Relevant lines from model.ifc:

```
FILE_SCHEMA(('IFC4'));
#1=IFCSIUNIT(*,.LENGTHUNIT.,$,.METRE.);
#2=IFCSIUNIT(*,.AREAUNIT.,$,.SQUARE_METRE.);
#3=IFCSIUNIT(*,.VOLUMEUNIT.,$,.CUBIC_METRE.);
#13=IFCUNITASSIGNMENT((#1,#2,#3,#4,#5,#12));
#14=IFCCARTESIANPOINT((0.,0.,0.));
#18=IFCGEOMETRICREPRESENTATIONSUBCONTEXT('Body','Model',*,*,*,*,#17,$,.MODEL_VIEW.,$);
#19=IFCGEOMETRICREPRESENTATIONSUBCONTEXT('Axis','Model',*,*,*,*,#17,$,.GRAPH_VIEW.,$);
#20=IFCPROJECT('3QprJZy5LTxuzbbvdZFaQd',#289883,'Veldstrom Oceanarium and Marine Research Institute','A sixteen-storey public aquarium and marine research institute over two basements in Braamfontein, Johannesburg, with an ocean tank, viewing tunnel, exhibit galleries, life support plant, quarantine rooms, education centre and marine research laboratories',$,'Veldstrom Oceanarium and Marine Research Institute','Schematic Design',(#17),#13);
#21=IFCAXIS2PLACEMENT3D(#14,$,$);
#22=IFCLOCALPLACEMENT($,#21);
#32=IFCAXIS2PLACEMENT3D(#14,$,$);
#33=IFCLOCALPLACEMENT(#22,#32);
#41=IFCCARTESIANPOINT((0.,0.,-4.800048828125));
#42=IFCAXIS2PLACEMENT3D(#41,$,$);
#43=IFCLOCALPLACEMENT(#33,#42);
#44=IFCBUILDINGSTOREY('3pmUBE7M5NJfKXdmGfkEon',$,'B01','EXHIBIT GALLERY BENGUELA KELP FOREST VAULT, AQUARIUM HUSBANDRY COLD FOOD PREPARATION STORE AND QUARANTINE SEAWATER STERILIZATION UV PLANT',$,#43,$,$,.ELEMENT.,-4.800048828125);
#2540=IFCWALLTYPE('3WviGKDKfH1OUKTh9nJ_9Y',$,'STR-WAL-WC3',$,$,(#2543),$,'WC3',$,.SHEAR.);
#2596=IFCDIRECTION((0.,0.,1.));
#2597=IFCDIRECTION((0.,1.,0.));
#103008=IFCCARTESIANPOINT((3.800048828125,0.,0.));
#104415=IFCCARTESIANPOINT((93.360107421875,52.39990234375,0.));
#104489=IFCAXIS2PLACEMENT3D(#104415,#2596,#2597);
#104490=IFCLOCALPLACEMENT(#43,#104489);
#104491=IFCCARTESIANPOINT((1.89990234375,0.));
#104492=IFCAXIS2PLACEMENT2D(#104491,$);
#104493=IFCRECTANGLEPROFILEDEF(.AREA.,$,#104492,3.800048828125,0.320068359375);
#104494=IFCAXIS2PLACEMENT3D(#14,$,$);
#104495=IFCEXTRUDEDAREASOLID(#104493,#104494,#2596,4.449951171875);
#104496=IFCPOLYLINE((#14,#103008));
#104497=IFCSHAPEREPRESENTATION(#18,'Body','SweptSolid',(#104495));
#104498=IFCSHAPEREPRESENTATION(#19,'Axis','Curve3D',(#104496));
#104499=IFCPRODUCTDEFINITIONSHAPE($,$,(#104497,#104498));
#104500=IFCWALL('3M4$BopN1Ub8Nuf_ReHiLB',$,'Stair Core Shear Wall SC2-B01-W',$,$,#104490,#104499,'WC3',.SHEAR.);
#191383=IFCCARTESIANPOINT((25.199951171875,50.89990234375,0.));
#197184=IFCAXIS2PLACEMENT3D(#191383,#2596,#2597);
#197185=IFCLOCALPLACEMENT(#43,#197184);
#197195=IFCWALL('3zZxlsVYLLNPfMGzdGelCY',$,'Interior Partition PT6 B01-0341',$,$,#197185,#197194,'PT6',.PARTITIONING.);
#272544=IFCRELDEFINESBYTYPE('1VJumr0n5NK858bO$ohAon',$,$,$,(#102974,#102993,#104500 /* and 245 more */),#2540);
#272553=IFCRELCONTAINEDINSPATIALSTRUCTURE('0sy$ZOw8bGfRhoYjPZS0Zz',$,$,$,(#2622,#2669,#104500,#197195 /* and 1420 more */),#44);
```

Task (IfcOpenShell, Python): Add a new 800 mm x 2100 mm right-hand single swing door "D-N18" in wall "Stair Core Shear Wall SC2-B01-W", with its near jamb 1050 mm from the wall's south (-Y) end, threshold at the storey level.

```python
import numpy as np
import ifcopenshell
import ifcopenshell.api.feature
import ifcopenshell.api.geometry
import ifcopenshell.api.root
import ifcopenshell.api.spatial
import ifcopenshell.geom
import ifcopenshell.util.element
import ifcopenshell.util.placement
import ifcopenshell.util.representation
import ifcopenshell.util.shape
import ifcopenshell.util.unit

model = ifcopenshell.open("model.ifc")
unit_scale = ifcopenshell.util.unit.calculate_unit_scale(model)
settings = ifcopenshell.geom.settings()


def volume(element):
    """Net volume in cubic metres, openings subtracted."""
    shape = ifcopenshell.geom.create_shape(settings, element)
    return ifcopenshell.util.shape.get_volume(shape.geometry)


wall = model.by_guid("3M4$BopN1Ub8Nuf_ReHiLB")
storey = ifcopenshell.util.element.get_container(wall, ifc_class="IfcBuildingStorey")
context = ifcopenshell.util.representation.get_context(model, "Model", "Body", "MODEL_VIEW")
before = volume(wall)

width, height, from_end, sill = 0.8, 2.1, 1.05, 0.0  # metres

# The wall runs along its own X axis, and the end named is its -X end.
wall_shape = ifcopenshell.geom.create_shape(settings, wall)
x, y, z = ifcopenshell.util.shape.get_vertices(wall_shape.geometry).T
start = x.min() + from_end
face, thickness = float(y.min()), float(y.max() - y.min())
wall_matrix = ifcopenshell.util.placement.get_local_placement(wall.ObjectPlacement)
level = ifcopenshell.util.placement.get_local_placement(storey.ObjectPlacement)[2, 3]


def in_wall(x, y):
    """Placement at x, y metres in the wall's axes, at sill height."""
    matrix = wall_matrix.copy()
    matrix[:, 3] = wall_matrix @ np.array([x / unit_scale, y / unit_scale, 0.0, 1.0])
    matrix[2, 3] = level + sill / unit_scale
    return matrix


# Opening: a box that overshoots both wall faces by 50 mm.
opening = ifcopenshell.api.root.create_entity(model, ifc_class="IfcOpeningElement", predefined_type="OPENING")
box = ifcopenshell.api.geometry.add_wall_representation(
    model, context=context, length=width, height=height, thickness=thickness + 0.1
)
ifcopenshell.api.geometry.assign_representation(model, product=opening, representation=box)
ifcopenshell.api.geometry.edit_object_placement(model, product=opening, matrix=in_wall(start, face - 0.05), is_si=False)
ifcopenshell.api.feature.add_feature(model, feature=opening, element=wall)

door = ifcopenshell.api.root.create_entity(model, ifc_class="IfcDoor", name="D-N18", predefined_type="DOOR")
door.OverallWidth, door.OverallHeight = width / unit_scale, height / unit_scale
door.OperationType = "SINGLE_SWING_RIGHT"
body = ifcopenshell.api.geometry.add_door_representation(
    model,
    context=context,
    overall_width=door.OverallWidth,
    overall_height=door.OverallHeight,
    operation_type="SINGLE_SWING_RIGHT",
    lining_properties={"LiningDepth": thickness / unit_scale, "ThresholdDepth": thickness / unit_scale},
)
ifcopenshell.api.geometry.assign_representation(model, product=door, representation=body)
ifcopenshell.api.spatial.assign_container(model, products=[door], relating_structure=storey)
ifcopenshell.api.feature.add_filling(model, opening=opening, element=door)

# The lining spans the wall, so the door starts at the wall face.
ifcopenshell.api.geometry.edit_object_placement(model, product=door, matrix=in_wall(start, face), is_si=False)

after = volume(wall)

print(f"wall volume {before:.3f} -> {after:.3f} m3")

model.write("model-out.ifc")
```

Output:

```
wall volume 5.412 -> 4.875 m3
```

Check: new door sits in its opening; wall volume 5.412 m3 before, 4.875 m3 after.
